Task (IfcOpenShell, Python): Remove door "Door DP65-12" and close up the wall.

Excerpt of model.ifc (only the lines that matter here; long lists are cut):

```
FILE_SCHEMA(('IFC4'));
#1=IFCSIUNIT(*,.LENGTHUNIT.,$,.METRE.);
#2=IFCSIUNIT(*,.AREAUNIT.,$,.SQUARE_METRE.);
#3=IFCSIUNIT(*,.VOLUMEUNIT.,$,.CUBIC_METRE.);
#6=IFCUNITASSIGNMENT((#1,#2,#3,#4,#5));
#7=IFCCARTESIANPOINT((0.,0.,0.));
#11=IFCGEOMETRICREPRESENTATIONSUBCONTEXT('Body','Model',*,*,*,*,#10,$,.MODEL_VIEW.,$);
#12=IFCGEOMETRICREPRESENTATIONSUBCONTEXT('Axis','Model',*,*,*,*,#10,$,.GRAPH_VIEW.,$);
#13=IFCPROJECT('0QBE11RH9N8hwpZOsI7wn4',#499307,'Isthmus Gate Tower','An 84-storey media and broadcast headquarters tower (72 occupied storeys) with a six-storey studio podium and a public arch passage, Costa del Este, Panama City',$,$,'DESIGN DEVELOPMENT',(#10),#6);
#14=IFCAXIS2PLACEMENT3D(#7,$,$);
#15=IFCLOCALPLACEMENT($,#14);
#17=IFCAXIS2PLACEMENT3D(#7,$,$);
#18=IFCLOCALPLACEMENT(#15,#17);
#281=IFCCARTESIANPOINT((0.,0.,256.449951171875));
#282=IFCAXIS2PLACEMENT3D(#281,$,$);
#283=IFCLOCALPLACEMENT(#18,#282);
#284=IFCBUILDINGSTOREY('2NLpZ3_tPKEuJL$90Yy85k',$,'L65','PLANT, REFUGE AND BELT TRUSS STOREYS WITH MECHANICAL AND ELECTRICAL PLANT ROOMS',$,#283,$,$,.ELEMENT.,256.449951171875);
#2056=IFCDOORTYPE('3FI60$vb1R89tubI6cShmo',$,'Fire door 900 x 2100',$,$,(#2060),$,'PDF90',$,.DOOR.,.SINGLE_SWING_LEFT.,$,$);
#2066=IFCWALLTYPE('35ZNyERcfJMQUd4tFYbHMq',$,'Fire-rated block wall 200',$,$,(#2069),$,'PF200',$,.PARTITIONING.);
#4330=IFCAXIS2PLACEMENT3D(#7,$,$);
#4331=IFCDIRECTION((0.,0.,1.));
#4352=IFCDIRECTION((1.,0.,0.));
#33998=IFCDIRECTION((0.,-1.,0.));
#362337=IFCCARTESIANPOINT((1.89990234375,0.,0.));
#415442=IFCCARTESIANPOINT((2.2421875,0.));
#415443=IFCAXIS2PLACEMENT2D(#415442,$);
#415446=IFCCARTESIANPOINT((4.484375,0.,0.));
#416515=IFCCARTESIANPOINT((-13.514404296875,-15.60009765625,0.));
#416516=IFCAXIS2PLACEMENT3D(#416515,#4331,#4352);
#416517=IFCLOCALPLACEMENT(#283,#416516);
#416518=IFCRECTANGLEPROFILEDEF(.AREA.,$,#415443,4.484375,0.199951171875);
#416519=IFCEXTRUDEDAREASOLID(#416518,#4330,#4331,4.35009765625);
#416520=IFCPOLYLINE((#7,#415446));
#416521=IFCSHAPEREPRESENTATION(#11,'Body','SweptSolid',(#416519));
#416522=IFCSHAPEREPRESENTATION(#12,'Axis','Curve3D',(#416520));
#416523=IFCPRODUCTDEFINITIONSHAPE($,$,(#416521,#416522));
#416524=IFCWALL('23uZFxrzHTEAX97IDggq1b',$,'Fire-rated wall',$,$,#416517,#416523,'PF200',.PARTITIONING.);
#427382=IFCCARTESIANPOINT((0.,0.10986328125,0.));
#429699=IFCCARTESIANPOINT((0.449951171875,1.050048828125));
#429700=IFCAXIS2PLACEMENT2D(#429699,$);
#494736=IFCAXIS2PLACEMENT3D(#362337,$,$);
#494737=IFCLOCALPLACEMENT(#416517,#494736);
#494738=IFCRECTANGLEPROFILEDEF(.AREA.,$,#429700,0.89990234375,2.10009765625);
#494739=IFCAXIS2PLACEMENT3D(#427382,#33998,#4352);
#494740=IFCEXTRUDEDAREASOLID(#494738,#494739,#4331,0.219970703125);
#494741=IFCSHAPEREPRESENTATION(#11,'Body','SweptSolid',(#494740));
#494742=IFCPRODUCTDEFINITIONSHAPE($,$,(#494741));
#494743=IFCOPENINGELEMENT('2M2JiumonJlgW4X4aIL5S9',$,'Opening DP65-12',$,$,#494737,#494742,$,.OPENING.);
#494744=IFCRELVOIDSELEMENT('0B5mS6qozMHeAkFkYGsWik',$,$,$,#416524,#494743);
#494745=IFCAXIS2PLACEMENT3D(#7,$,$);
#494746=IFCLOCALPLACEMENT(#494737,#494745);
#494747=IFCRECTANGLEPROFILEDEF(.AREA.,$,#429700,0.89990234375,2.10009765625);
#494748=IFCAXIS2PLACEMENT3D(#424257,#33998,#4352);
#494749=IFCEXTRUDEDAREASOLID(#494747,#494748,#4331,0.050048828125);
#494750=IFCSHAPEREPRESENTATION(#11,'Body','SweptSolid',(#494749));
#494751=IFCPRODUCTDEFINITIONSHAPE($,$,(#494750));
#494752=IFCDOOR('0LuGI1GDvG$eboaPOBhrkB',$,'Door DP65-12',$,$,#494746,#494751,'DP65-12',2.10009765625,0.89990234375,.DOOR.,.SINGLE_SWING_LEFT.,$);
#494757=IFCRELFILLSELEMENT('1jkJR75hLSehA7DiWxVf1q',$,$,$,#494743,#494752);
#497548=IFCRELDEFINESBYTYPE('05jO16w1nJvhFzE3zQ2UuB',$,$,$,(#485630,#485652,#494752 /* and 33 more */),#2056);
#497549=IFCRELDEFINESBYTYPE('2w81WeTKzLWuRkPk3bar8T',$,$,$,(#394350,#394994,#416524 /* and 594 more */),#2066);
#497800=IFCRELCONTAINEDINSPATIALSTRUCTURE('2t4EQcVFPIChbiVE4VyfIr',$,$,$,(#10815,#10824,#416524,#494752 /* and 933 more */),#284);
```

```python
import ifcopenshell
import ifcopenshell.api.feature
import ifcopenshell.api.root
import ifcopenshell.geom
import ifcopenshell.util.shape

model = ifcopenshell.open("model.ifc")
settings = ifcopenshell.geom.settings()


def volume(element):
    """Net volume in cubic metres, openings subtracted."""
    shape = ifcopenshell.geom.create_shape(settings, element)
    return ifcopenshell.util.shape.get_volume(shape.geometry)


door = model.by_id(494752)
opening = door.FillsVoids[0].RelatingOpeningElement
wall = opening.VoidsElements[0].RelatingBuildingElement
before = volume(wall)

ifcopenshell.api.root.remove_product(model, product=door)
ifcopenshell.api.feature.remove_feature(model, feature=opening)

after = volume(wall)

print(f"wall volume {before:.3f} -> {after:.3f} m3")

model.write("model_updated.ifc")
```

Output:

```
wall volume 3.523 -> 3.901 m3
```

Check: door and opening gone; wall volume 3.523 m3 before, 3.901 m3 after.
